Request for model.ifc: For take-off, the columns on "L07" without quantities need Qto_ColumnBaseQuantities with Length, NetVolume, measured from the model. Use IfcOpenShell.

First a look at what the model holds.

```python
import ifcopenshell
import ifcopenshell.util.element
import ifcopenshell.util.unit

model = ifcopenshell.open("model.ifc")
print(model.schema)
for unit_type in ("LENGTHUNIT", "AREAUNIT", "VOLUMEUNIT"):
    print(unit_type, ifcopenshell.util.unit.calculate_unit_scale(model, unit_type))
storey = next(s for s in model.by_type("IfcBuildingStorey") if s.Name == "L07")
columns = [e for e in ifcopenshell.util.element.get_decomposition(storey) if e.is_a("IfcColumn")]
for e in sorted(columns, key=lambda e: e.id()):
    print(e.id(), e.is_a(), e.Name, list(ifcopenshell.util.element.get_psets(e, qtos_only=True)), sep=" | ")
```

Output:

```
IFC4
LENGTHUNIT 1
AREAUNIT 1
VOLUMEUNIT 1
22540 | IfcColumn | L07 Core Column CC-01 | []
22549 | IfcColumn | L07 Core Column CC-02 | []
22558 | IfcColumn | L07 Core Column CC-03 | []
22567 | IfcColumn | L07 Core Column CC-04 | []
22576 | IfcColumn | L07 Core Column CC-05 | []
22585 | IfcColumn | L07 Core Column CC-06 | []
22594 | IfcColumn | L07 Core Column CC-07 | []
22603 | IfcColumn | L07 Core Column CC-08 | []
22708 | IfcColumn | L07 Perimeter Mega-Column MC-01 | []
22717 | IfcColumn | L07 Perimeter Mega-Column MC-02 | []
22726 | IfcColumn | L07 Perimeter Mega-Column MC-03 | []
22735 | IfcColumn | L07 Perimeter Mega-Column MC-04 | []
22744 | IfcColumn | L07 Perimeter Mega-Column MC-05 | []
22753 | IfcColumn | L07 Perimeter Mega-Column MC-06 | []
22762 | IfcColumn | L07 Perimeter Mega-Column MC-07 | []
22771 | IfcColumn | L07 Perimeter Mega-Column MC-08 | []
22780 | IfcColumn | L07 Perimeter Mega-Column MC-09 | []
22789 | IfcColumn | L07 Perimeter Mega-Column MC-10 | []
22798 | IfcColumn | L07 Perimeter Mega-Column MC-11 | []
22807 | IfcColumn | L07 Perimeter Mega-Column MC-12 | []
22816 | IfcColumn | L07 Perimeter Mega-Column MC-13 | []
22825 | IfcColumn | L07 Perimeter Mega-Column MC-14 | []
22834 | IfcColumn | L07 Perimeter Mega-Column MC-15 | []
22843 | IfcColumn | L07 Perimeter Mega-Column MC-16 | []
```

```python
import ifcopenshell
import ifcopenshell.api.pset
import ifcopenshell.geom
import ifcopenshell.util.element
import ifcopenshell.util.shape
import ifcopenshell.util.unit

model = ifcopenshell.open("model.ifc")
unit_scale = ifcopenshell.util.unit.calculate_unit_scale(model)
volume_scale = ifcopenshell.util.unit.calculate_unit_scale(model, "VOLUMEUNIT")
settings = ifcopenshell.geom.settings()

storey = next(s for s in model.by_type("IfcBuildingStorey") if s.Name == "L07")
columns = [e for e in ifcopenshell.util.element.get_decomposition(storey) if e.is_a("IfcColumn")]

for e in sorted(columns, key=lambda e: e.id()):
    if ifcopenshell.util.element.get_psets(e, qtos_only=True, should_inherit=False):
        continue
    # Geometry comes back in metres, in the element's own axes.
    shape = ifcopenshell.geom.create_shape(settings, e)
    values = {
        "Length": ifcopenshell.util.shape.get_z(shape.geometry) / unit_scale,
        "NetVolume": ifcopenshell.util.shape.get_volume(shape.geometry) / volume_scale,
    }
    qto = ifcopenshell.api.pset.add_qto(model, product=e, name="Qto_ColumnBaseQuantities")
    ifcopenshell.api.pset.edit_qto(model, qto=qto, properties=values)
    print(e.id(), {k: round(v, 3) for k, v in values.items()})

model.write("model_updated.ifc")
```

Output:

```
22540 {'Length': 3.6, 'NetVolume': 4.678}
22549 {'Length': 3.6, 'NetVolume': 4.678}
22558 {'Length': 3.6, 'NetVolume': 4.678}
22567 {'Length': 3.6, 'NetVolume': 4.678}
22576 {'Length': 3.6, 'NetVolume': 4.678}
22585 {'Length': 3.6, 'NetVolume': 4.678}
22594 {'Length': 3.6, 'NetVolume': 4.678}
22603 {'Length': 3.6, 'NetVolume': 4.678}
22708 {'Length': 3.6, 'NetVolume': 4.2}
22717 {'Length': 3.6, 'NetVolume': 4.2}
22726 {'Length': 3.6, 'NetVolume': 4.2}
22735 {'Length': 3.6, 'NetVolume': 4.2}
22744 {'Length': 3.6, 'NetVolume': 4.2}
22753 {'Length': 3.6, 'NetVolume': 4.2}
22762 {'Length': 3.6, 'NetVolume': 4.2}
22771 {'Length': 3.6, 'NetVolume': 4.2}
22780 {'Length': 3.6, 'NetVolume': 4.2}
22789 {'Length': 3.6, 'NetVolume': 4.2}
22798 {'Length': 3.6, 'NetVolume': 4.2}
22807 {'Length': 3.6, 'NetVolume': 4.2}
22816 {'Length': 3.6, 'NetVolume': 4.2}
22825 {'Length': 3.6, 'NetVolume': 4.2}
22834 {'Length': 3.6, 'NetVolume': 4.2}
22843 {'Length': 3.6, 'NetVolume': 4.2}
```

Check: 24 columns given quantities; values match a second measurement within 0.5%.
